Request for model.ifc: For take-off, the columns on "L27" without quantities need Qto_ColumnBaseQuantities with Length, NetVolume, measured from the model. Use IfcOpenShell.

First a look at what the model holds.

```python
import ifcopenshell
import ifcopenshell.util.element
import ifcopenshell.util.unit

model = ifcopenshell.open("model.ifc")
print(model.schema)
for unit_type in ("LENGTHUNIT", "AREAUNIT", "VOLUMEUNIT"):
    print(unit_type, ifcopenshell.util.unit.calculate_unit_scale(model, unit_type))
storey = next(s for s in model.by_type("IfcBuildingStorey") if s.Name == "L27")
columns = [e for e in ifcopenshell.util.element.get_decomposition(storey) if e.is_a("IfcColumn")]
for e in sorted(columns, key=lambda e: e.id()):
    print(e.id(), e.is_a(), e.Name, list(ifcopenshell.util.element.get_psets(e, qtos_only=True)), sep=" | ")
```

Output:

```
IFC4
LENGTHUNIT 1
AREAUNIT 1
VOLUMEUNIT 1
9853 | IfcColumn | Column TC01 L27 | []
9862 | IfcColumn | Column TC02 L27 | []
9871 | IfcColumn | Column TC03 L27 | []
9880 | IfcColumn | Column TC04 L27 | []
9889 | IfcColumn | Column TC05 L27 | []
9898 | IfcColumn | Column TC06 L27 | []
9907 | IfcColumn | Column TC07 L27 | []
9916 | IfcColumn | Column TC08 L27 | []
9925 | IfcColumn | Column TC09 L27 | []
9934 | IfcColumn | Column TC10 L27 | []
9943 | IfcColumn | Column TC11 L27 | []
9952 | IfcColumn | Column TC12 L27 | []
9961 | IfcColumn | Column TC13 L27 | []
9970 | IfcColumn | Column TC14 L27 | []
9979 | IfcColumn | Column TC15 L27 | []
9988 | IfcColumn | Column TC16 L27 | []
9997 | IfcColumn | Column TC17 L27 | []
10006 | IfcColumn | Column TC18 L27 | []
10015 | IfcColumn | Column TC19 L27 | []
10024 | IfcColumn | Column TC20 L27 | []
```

```python
import ifcopenshell
import ifcopenshell.api.pset
import ifcopenshell.geom
import ifcopenshell.util.element
import ifcopenshell.util.shape
import ifcopenshell.util.unit

model = ifcopenshell.open("model.ifc")
unit_scale = ifcopenshell.util.unit.calculate_unit_scale(model)
volume_scale = ifcopenshell.util.unit.calculate_unit_scale(model, "VOLUMEUNIT")
settings = ifcopenshell.geom.settings()

storey = next(s for s in model.by_type("IfcBuildingStorey") if s.Name == "L27")
columns = [e for e in ifcopenshell.util.element.get_decomposition(storey) if e.is_a("IfcColumn")]

for e in sorted(columns, key=lambda e: e.id()):
    if ifcopenshell.util.element.get_psets(e, qtos_only=True, should_inherit=False):
        continue
    # Geometry comes back in metres, in the element's own axes.
    shape = ifcopenshell.geom.create_shape(settings, e)
    values = {
        "Length": ifcopenshell.util.shape.get_z(shape.geometry) / unit_scale,
        "NetVolume": ifcopenshell.util.shape.get_volume(shape.geometry) / volume_scale,
    }
    qto = ifcopenshell.api.pset.add_qto(model, product=e, name="Qto_ColumnBaseQuantities")
    ifcopenshell.api.pset.edit_qto(model, qto=qto, properties=values)
    print(e.id(), {k: round(v, 3) for k, v in values.items()})

model.write("model_updated.ifc")
```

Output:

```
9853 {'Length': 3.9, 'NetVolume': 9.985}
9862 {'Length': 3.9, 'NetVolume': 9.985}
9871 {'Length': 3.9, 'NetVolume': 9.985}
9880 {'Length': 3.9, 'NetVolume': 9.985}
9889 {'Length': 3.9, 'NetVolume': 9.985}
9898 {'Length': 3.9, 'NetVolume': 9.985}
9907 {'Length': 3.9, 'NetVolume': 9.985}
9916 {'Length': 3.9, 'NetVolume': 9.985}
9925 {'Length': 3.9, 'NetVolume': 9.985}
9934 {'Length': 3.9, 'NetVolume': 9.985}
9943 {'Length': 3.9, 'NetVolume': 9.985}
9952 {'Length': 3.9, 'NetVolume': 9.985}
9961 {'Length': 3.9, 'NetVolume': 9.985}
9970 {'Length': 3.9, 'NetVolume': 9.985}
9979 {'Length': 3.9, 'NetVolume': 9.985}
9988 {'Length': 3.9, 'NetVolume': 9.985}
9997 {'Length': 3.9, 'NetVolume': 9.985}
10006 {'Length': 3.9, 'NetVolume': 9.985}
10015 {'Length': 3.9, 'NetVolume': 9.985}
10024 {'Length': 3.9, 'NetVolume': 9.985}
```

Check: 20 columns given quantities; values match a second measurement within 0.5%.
